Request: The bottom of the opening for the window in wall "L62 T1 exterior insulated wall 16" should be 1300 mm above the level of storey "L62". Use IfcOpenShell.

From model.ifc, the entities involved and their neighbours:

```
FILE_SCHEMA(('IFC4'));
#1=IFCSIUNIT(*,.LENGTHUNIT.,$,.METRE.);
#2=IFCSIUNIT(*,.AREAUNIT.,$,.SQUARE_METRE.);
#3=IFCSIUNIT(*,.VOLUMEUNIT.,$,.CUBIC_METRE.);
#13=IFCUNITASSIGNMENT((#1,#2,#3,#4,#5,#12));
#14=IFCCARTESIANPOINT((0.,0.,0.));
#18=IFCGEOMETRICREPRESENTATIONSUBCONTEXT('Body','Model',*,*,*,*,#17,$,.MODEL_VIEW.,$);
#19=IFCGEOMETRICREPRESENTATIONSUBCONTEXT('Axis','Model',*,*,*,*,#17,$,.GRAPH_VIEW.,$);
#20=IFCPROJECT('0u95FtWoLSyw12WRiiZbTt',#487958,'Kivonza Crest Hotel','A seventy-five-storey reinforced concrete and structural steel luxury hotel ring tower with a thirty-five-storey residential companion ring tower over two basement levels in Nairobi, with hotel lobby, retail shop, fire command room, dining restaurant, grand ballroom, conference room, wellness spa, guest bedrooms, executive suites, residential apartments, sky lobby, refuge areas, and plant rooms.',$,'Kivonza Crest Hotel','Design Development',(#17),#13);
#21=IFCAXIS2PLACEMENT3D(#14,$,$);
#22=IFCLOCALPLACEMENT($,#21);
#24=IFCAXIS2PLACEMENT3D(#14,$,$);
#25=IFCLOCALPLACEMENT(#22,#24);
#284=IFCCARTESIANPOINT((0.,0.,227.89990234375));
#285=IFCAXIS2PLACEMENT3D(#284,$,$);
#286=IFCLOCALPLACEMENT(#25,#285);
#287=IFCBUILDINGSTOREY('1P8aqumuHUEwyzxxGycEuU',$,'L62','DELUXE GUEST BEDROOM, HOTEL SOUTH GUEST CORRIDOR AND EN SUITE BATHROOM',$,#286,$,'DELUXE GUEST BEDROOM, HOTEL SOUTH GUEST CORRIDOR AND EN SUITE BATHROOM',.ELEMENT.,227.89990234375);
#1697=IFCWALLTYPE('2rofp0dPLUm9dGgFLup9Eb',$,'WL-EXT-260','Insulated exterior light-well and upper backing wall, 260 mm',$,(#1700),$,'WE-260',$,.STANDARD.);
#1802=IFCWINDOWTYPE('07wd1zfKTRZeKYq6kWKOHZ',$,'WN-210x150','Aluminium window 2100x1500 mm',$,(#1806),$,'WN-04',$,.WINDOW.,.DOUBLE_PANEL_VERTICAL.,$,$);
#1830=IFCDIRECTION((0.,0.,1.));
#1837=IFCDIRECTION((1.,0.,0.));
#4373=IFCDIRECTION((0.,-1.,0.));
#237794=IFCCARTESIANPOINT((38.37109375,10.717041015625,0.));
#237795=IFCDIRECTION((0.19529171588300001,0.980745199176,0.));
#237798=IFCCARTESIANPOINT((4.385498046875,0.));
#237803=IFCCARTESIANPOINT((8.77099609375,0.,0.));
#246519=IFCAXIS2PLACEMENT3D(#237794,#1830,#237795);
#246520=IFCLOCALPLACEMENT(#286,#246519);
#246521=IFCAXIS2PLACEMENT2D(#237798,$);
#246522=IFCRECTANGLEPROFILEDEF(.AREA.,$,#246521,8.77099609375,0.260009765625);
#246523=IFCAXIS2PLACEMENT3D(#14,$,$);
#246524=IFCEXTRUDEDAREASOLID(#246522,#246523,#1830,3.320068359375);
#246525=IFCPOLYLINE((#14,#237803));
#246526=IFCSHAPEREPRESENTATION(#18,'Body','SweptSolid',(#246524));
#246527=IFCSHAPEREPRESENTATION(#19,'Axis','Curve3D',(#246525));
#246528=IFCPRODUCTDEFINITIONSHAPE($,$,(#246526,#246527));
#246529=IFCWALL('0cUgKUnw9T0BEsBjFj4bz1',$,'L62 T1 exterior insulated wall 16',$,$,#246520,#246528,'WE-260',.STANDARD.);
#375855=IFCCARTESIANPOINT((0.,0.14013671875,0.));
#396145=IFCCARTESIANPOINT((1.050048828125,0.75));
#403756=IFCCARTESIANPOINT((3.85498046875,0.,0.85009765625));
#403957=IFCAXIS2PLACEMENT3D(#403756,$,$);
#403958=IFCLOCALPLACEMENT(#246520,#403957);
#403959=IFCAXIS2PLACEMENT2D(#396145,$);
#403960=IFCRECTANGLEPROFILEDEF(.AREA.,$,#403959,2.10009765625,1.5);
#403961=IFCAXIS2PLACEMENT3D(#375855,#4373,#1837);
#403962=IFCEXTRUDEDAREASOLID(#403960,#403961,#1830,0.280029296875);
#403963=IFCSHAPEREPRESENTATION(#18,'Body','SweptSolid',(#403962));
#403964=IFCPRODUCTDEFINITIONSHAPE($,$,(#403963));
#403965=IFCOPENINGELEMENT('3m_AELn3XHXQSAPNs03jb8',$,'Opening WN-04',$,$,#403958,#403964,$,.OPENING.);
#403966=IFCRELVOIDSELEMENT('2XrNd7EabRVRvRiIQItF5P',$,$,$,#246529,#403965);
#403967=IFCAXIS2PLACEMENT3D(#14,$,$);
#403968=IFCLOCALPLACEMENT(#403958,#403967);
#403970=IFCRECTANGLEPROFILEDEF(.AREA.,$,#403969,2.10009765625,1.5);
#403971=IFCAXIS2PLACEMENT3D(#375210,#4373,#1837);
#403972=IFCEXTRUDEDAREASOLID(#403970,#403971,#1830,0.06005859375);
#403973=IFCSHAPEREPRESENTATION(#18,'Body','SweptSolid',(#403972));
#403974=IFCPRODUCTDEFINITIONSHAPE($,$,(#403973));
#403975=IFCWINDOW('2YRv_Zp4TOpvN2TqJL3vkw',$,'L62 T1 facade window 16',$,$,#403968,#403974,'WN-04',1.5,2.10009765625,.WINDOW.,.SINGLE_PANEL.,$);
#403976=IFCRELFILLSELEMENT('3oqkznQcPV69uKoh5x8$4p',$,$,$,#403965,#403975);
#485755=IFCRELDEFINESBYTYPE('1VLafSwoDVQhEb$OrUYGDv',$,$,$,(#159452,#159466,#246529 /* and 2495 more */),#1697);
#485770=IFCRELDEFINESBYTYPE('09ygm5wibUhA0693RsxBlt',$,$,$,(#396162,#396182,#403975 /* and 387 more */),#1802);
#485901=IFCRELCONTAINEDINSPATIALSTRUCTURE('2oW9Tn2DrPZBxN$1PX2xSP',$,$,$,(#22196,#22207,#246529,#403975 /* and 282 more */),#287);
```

```python
import numpy as np
import ifcopenshell
import ifcopenshell.api.geometry
import ifcopenshell.geom
import ifcopenshell.util.element
import ifcopenshell.util.placement
import ifcopenshell.util.shape
import ifcopenshell.util.unit

model = ifcopenshell.open("model.ifc")
unit_scale = ifcopenshell.util.unit.calculate_unit_scale(model)

window = model.by_guid("2YRv_Zp4TOpvN2TqJL3vkw")
opening = window.FillsVoids[0].RelatingOpeningElement
storey = ifcopenshell.util.element.get_container(window, ifc_class="IfcBuildingStorey")
level = ifcopenshell.util.placement.get_local_placement(storey.ObjectPlacement)[2, 3]

# The opening's origin need not be at the sill, so measure its lowest point.
shape = ifcopenshell.geom.create_shape(ifcopenshell.geom.settings(), opening)
bottom = ifcopenshell.util.shape.get_shape_bottom_elevation(shape, shape.geometry) / unit_scale
dz = level + 1.3 / unit_scale - bottom

shift = np.array([0.0, 0.0, dz])
# The window is placed relative to its opening, so it follows when the opening moves.
matrix = ifcopenshell.util.placement.get_local_placement(opening.ObjectPlacement)
matrix[:3, 3] += shift
ifcopenshell.api.geometry.edit_object_placement(
    model, product=opening, matrix=matrix, is_si=False, should_transform_children=True
)

print(f"moved by {dz * unit_scale:+.3f} m")

model.write("model_updated.ifc")
```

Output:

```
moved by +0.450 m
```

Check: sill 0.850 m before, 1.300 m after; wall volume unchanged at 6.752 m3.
